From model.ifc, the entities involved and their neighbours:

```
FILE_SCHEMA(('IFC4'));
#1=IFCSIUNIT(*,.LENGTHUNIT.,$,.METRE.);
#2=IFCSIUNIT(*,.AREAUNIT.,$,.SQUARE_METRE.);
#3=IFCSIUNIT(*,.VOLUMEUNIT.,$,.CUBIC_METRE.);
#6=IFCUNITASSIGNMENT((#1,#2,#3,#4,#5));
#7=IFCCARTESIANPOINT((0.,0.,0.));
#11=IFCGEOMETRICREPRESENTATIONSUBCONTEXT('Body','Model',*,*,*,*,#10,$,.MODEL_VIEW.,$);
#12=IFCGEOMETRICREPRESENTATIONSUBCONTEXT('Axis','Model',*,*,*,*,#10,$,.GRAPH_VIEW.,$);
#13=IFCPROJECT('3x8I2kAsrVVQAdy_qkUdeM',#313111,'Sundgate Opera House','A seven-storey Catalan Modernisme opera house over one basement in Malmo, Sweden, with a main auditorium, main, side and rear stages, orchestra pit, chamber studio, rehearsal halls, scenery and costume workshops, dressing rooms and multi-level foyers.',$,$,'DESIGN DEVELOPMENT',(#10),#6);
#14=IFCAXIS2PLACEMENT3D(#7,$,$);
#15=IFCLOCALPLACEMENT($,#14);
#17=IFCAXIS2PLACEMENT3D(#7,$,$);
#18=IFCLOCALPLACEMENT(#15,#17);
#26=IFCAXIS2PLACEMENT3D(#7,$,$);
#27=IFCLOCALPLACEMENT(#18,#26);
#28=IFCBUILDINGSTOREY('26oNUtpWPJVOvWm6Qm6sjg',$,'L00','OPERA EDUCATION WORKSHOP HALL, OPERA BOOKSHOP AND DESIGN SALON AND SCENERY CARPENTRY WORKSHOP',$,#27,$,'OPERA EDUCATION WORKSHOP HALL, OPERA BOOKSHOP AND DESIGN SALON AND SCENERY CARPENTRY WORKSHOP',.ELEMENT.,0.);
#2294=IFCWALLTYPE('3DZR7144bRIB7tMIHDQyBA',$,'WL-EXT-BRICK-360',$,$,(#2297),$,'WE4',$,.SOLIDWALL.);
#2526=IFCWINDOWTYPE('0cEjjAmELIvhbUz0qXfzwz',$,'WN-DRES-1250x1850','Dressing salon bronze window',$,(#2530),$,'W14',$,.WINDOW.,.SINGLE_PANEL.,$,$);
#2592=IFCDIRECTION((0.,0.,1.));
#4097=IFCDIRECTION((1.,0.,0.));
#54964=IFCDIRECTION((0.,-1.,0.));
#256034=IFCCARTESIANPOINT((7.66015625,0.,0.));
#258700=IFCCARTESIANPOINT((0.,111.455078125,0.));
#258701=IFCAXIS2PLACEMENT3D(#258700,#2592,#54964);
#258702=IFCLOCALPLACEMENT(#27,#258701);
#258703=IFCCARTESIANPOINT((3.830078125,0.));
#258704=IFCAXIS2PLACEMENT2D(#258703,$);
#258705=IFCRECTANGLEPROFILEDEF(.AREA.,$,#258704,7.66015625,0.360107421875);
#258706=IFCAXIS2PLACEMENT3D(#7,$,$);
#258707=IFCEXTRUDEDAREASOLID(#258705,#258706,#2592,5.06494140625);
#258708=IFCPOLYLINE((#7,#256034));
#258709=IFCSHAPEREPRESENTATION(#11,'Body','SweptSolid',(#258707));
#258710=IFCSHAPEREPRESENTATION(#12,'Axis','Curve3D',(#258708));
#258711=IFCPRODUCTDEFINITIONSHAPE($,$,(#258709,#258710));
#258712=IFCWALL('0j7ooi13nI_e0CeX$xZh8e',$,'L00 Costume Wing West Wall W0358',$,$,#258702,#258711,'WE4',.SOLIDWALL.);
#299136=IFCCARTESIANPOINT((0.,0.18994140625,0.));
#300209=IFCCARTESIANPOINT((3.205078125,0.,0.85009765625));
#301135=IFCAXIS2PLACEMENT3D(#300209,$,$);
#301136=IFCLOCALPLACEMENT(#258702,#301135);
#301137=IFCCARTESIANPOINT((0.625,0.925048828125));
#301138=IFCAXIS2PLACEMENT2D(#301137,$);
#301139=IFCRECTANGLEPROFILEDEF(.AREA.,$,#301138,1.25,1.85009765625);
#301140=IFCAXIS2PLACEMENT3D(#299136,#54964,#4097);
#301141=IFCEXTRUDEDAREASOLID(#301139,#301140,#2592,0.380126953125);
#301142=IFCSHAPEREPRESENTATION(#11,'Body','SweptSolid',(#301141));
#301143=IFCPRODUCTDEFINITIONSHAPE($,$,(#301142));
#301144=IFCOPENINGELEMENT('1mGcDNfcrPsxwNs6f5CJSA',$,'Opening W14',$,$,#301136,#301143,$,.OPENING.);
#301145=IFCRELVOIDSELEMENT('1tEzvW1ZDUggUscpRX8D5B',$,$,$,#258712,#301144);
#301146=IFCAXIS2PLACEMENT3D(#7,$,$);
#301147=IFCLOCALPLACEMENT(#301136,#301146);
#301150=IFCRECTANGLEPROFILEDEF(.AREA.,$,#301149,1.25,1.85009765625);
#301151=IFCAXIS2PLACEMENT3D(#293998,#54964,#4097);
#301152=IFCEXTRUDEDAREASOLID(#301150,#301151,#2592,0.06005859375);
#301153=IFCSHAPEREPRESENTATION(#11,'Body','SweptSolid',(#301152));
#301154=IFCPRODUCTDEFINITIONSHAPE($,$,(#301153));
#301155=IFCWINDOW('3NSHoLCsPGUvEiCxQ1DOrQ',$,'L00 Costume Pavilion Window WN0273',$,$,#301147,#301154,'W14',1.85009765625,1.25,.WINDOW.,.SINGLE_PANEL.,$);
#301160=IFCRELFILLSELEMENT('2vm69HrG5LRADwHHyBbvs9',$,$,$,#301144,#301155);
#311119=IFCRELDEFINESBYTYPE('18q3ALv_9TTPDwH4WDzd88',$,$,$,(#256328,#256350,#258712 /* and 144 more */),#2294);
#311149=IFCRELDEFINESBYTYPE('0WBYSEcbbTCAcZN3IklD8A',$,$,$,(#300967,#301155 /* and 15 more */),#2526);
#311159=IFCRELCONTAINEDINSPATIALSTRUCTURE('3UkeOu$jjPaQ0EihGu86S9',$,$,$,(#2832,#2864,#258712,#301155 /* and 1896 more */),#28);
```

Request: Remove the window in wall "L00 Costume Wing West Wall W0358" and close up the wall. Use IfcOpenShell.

```python
import ifcopenshell
import ifcopenshell.api.feature
import ifcopenshell.api.root
import ifcopenshell.geom
import ifcopenshell.util.shape

model = ifcopenshell.open("model.ifc")
settings = ifcopenshell.geom.settings()


def volume(element):
    """Net volume in cubic metres, openings subtracted."""
    shape = ifcopenshell.geom.create_shape(settings, element)
    return ifcopenshell.util.shape.get_volume(shape.geometry)


window = model.by_guid("3NSHoLCsPGUvEiCxQ1DOrQ")
opening = window.FillsVoids[0].RelatingOpeningElement
wall = opening.VoidsElements[0].RelatingBuildingElement
before = volume(wall)

ifcopenshell.api.root.remove_product(model, product=window)
ifcopenshell.api.feature.remove_feature(model, feature=opening)

after = volume(wall)

print(f"wall volume {before:.3f} -> {after:.3f} m3")

model.write("model_edited.ifc")
```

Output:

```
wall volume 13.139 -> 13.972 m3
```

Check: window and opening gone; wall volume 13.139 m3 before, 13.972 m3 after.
